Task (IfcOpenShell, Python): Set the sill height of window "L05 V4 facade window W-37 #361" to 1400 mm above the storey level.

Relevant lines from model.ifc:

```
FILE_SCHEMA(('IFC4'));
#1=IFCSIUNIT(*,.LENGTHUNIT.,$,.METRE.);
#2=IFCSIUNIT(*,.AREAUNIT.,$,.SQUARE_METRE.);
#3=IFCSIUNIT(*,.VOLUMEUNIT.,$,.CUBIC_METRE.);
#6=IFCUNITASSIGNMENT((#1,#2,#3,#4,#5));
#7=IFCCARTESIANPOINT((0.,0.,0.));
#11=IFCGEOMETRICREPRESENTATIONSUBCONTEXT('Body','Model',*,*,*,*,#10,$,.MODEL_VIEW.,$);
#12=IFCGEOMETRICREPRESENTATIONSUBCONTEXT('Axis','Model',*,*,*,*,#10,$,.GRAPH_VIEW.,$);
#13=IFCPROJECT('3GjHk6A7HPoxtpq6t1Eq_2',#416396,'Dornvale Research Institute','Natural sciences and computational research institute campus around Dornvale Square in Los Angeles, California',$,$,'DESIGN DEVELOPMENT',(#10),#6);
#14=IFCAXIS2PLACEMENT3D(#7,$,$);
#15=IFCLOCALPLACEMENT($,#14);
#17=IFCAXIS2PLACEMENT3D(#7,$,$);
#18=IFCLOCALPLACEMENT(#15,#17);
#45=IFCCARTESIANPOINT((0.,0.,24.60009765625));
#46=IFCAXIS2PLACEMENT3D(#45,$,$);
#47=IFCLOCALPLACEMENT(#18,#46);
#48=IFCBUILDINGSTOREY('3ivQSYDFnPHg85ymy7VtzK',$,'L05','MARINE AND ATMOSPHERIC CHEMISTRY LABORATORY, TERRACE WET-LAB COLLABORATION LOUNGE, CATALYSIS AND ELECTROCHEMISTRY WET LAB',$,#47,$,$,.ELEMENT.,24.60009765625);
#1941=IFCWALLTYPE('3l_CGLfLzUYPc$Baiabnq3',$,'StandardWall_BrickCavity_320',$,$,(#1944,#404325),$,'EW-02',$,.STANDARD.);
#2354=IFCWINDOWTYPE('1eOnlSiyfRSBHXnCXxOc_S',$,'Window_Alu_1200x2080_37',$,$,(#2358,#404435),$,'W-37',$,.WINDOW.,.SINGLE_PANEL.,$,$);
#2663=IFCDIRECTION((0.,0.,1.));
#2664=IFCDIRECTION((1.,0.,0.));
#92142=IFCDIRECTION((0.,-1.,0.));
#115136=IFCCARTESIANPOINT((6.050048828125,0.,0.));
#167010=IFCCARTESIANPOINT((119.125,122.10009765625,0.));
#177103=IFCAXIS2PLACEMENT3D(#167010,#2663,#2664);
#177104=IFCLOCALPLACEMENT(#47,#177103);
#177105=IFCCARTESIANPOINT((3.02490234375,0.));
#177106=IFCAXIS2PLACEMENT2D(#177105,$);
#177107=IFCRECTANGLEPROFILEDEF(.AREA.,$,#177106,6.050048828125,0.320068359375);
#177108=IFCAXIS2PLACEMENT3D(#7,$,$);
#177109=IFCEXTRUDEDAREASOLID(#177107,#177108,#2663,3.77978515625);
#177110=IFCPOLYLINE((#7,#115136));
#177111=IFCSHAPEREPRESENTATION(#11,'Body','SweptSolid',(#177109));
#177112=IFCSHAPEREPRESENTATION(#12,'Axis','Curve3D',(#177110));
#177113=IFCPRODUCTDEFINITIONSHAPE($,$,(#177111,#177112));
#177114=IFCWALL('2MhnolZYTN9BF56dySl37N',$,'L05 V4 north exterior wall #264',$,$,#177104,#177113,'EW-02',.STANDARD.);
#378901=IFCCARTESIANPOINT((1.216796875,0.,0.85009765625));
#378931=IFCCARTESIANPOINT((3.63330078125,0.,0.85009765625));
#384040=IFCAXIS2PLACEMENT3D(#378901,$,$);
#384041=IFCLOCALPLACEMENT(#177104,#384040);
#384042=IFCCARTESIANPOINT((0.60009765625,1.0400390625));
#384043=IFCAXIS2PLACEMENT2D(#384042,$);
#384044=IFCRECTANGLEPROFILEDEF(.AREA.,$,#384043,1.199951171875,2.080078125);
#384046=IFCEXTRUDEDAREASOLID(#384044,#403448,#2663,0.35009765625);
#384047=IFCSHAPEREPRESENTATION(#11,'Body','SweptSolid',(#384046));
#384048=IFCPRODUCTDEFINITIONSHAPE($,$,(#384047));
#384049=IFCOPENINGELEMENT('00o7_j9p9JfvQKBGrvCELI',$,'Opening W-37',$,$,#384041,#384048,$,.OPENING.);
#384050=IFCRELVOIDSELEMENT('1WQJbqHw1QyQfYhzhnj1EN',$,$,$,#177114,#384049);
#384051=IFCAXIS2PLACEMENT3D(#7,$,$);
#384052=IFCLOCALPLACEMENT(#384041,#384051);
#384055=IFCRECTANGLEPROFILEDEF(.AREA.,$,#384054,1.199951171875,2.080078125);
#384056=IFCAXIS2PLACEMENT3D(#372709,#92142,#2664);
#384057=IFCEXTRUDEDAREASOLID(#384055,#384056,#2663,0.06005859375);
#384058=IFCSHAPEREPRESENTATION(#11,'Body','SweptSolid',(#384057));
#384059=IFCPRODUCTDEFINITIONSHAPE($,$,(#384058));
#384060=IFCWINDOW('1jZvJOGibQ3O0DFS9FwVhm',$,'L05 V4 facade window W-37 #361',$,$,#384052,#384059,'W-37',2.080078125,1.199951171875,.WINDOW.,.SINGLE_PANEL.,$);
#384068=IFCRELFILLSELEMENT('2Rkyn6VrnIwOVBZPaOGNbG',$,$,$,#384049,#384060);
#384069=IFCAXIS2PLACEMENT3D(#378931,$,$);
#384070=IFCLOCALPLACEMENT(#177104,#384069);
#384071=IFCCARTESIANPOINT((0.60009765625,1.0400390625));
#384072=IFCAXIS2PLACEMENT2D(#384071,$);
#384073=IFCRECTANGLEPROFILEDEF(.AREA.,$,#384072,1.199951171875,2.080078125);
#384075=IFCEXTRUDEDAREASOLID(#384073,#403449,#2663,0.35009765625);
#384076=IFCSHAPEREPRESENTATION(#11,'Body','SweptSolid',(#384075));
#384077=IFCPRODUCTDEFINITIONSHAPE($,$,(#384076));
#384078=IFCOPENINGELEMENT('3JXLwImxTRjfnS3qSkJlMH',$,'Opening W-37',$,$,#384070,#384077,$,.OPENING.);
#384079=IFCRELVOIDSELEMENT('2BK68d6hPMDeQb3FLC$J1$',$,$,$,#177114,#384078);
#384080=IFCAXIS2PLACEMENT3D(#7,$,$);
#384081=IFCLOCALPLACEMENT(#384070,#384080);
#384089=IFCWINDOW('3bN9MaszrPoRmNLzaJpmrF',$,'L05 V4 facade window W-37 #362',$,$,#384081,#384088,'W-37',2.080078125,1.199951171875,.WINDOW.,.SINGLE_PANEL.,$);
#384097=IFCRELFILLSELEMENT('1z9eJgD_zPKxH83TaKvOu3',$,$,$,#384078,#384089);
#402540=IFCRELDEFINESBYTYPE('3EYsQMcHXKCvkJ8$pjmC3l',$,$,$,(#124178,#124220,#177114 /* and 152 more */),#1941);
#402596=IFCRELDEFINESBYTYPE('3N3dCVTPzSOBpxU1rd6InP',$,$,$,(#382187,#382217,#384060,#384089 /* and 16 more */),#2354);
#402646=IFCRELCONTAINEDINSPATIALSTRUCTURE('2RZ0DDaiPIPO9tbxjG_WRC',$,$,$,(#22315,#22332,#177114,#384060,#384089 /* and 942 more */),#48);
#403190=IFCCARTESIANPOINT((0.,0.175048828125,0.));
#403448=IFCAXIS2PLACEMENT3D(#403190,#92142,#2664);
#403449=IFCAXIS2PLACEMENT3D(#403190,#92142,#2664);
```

```python
import numpy as np
import ifcopenshell
import ifcopenshell.api.geometry
import ifcopenshell.geom
import ifcopenshell.util.element
import ifcopenshell.util.placement
import ifcopenshell.util.shape
import ifcopenshell.util.unit

model = ifcopenshell.open("model.ifc")
unit_scale = ifcopenshell.util.unit.calculate_unit_scale(model)

window = model.by_guid("1jZvJOGibQ3O0DFS9FwVhm")
opening = window.FillsVoids[0].RelatingOpeningElement
storey = ifcopenshell.util.element.get_container(window, ifc_class="IfcBuildingStorey")
level = ifcopenshell.util.placement.get_local_placement(storey.ObjectPlacement)[2, 3]

# The opening's origin need not be at the sill, so measure its lowest point.
shape = ifcopenshell.geom.create_shape(ifcopenshell.geom.settings(), opening)
bottom = ifcopenshell.util.shape.get_shape_bottom_elevation(shape, shape.geometry) / unit_scale
dz = level + 1.4 - bottom

shift = np.array([0.0, 0.0, dz])
# The window is placed relative to its opening, so it follows when the opening moves.
matrix = ifcopenshell.util.placement.get_local_placement(opening.ObjectPlacement)
matrix[:3, 3] += shift
ifcopenshell.api.geometry.edit_object_placement(
    model, product=opening, matrix=matrix, is_si=False, should_transform_children=True
)

print(f"moved by {dz * unit_scale:+.3f} m")

model.write("model-out.ifc")
```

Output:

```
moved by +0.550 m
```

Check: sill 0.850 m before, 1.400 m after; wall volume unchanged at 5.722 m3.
